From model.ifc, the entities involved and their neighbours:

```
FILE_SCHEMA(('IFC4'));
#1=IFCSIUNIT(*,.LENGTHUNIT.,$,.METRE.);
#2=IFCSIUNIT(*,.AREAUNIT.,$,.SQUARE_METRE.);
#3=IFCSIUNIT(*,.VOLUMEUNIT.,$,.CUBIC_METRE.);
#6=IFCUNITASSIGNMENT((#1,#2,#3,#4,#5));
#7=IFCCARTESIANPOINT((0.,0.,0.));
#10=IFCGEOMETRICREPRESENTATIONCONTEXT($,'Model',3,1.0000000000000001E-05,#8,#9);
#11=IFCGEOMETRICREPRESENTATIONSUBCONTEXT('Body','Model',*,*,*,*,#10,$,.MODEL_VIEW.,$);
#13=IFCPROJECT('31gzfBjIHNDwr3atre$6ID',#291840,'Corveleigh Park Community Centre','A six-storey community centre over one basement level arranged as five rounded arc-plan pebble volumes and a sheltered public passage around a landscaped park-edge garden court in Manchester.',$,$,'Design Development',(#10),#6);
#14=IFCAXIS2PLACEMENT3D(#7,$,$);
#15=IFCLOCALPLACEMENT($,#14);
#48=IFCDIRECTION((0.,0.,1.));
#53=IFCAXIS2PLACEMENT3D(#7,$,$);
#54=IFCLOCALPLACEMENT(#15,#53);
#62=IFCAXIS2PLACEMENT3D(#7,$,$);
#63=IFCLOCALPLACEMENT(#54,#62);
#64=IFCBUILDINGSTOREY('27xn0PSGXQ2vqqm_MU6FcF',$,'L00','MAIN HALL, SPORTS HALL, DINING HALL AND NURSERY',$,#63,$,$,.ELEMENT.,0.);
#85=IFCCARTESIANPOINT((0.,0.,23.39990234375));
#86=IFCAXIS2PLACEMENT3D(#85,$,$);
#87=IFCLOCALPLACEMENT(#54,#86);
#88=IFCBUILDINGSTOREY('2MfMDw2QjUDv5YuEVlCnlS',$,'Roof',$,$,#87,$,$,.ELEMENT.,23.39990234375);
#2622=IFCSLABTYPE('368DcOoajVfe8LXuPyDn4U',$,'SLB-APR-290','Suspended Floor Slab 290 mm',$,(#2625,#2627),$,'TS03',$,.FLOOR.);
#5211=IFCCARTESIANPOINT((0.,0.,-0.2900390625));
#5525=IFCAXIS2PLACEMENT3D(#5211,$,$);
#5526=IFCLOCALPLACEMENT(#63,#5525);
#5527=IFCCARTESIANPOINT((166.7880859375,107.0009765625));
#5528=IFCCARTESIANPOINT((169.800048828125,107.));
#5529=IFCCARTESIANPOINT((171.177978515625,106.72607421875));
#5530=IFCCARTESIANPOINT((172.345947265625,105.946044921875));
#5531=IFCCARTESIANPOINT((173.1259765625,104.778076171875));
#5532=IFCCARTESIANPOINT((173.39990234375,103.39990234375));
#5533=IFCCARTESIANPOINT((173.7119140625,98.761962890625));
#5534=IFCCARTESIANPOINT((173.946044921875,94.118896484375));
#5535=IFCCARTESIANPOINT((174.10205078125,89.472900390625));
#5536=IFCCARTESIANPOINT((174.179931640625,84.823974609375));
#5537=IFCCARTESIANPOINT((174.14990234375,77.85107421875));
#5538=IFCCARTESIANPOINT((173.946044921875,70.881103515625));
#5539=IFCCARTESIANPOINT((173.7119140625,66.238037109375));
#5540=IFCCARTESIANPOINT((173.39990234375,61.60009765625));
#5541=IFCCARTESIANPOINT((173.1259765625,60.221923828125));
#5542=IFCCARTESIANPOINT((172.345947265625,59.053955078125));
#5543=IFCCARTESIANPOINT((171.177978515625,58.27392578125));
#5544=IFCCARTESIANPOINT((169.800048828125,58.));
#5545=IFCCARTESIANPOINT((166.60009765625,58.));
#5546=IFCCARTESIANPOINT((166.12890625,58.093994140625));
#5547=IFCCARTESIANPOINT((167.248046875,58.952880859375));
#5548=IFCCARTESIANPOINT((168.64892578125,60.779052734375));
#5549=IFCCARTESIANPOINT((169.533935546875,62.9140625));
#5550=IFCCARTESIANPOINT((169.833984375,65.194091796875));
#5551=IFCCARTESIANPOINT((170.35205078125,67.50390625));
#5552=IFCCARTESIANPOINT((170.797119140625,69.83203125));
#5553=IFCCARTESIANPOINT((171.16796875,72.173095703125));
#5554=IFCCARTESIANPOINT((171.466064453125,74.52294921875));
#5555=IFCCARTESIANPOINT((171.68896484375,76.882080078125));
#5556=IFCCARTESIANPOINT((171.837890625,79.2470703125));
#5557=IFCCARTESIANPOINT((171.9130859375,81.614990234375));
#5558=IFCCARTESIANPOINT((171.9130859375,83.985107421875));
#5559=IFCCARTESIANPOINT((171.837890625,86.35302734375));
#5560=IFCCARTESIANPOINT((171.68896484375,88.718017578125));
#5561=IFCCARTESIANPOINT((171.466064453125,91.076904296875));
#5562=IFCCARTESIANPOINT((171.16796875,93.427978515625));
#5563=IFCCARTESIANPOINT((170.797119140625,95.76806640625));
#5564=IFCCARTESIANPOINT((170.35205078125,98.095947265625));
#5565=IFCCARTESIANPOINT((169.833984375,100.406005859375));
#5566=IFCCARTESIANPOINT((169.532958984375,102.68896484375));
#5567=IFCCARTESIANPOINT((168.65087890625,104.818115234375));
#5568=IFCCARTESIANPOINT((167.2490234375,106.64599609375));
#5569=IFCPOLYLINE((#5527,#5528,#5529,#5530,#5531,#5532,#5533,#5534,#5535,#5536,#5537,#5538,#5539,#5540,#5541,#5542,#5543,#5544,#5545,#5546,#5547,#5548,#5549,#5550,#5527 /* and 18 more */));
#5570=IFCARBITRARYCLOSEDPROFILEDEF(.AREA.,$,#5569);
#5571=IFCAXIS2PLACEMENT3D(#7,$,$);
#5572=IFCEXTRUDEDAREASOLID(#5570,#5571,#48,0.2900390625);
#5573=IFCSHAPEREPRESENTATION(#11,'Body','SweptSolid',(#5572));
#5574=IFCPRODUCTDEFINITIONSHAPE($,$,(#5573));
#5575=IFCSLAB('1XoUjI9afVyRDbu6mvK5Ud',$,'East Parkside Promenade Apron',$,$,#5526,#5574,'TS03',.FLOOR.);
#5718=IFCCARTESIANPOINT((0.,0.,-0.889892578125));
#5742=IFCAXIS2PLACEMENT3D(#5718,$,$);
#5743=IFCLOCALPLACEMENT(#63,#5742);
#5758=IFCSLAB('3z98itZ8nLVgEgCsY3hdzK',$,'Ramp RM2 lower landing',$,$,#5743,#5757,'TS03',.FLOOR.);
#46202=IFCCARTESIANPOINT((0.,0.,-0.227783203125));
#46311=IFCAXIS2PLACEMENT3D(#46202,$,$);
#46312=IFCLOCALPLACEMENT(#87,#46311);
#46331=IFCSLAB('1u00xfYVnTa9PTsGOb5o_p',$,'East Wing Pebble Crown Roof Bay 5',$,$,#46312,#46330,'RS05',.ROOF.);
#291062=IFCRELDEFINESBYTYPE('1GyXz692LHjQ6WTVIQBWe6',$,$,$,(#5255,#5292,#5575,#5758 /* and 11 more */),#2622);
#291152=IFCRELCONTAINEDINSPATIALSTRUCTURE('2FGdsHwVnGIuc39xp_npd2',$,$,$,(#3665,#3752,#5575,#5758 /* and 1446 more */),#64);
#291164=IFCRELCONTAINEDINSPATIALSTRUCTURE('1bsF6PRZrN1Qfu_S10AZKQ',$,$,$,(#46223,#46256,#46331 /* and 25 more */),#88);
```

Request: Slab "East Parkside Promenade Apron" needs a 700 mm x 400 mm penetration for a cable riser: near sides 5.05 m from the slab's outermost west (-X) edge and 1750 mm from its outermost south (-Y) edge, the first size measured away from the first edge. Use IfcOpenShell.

```python
import numpy as np
import ifcopenshell
import ifcopenshell.api.feature
import ifcopenshell.api.geometry
import ifcopenshell.api.root
import ifcopenshell.geom
import ifcopenshell.util.placement
import ifcopenshell.util.representation
import ifcopenshell.util.shape
import ifcopenshell.util.unit

model = ifcopenshell.open("model.ifc")
unit_scale = ifcopenshell.util.unit.calculate_unit_scale(model)
settings = ifcopenshell.geom.settings()


def volume(element):
    """Net volume in cubic metres, openings subtracted."""
    shape = ifcopenshell.geom.create_shape(settings, element)
    return ifcopenshell.util.shape.get_volume(shape.geometry)


slab = model.by_guid("1XoUjI9afVyRDbu6mvK5Ud")
before = volume(slab)

# Extent in the slab's own axes, in metres. The edges named are its -X and -Y sides.
slab_shape = ifcopenshell.geom.create_shape(settings, slab)
vertices = ifcopenshell.util.shape.get_vertices(slab_shape.geometry)
x_min, y_min, bottom = vertices.min(axis=0)
top = vertices[:, 2].max()

opening = ifcopenshell.api.root.create_entity(model, ifc_class="IfcOpeningElement", name="Cable riser opening", predefined_type="OPENING")
context = ifcopenshell.util.representation.get_context(model, "Model", "Body", "MODEL_VIEW")
width, depth = 0.7, 0.4
outline = [(0.0, 0.0), (width, 0.0), (width, depth), (0.0, depth), (0.0, 0.0)]
# Overshoot both faces by 50 mm so the cut is clean.
shape = ifcopenshell.api.geometry.add_slab_representation(
    model, context=context, depth=top - bottom + 0.1, polyline=outline
)
ifcopenshell.api.geometry.assign_representation(model, product=opening, representation=shape)

matrix = ifcopenshell.util.placement.get_local_placement(slab.ObjectPlacement)
matrix[:, 3] = matrix @ np.append(np.array([x_min + 5.05, y_min + 1.75, bottom - 0.05]) / unit_scale, 1.0)
ifcopenshell.api.geometry.edit_object_placement(model, product=opening, matrix=matrix, is_si=False)
ifcopenshell.api.feature.add_feature(model, feature=opening, element=slab)

after = volume(slab)

print(f"slab volume {before:.3f} -> {after:.3f} m3")

model.write("model_updated.ifc")
```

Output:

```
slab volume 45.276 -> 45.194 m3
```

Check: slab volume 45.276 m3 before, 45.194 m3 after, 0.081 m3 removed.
